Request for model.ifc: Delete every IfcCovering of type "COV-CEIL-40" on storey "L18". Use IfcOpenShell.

First a look at what the model holds.

```python
import ifcopenshell
import ifcopenshell.util.element

model = ifcopenshell.open("model.ifc")
print(model.schema)
storey = next(s for s in model.by_type("IfcBuildingStorey") if s.Name == "L18")
coverings = [e for e in ifcopenshell.util.element.get_decomposition(storey) if e.is_a("IfcCovering")]
seen = {}
for e in coverings:
    element_type = ifcopenshell.util.element.get_type(e)
    name = element_type.Name if element_type not in (None, e) else None
    seen[name] = seen.get(name, 0) + 1
for name, count in sorted(seen.items(), key=str):
    print(count, "x", name)
```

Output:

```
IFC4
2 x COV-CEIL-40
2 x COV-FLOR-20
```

```python
import ifcopenshell
import ifcopenshell.api.root
import ifcopenshell.util.element

model = ifcopenshell.open("model.ifc")

storey = next(s for s in model.by_type("IfcBuildingStorey") if s.Name == "L18")
coverings = [e for e in ifcopenshell.util.element.get_decomposition(storey) if e.is_a("IfcCovering")]
targets = [e for e in coverings if (t := ifcopenshell.util.element.get_type(e)) not in (None, e) and t.Name == "COV-CEIL-40"]

for e in targets:
    ifcopenshell.api.root.remove_product(model, product=e)
print(len(targets), "removed")

model.write("model_rev.ifc")
```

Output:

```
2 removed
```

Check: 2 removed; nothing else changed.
